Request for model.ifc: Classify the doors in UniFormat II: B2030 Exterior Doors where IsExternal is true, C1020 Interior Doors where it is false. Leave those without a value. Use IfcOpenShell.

First a look at what the model holds.

```python
import ifcopenshell
import ifcopenshell.util.element

model = ifcopenshell.open("model.ifc")
print(model.schema)
print("classifications:", [c.Name for c in model.by_type("IfcClassification")])
values = [ifcopenshell.util.element.get_pset(e, "Pset_DoorCommon", "IsExternal") for e in model.by_type("IfcDoor")]
for value in (True, False, None):
    print("IsExternal", value, values.count(value))
```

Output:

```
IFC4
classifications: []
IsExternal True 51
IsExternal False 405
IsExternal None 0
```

```python
import ifcopenshell
import ifcopenshell.api.classification
import ifcopenshell.util.element

model = ifcopenshell.open("model.ifc")

system = ifcopenshell.api.classification.add_classification(model, classification="UniFormat II")

doors = model.by_type("IfcDoor")
external = {e: ifcopenshell.util.element.get_pset(e, "Pset_DoorCommon", "IsExternal") for e in doors}
for flag, code, name in ((True, "B2030", "Exterior Doors"), (False, "C1020", "Interior Doors")):
    products = [e for e in doors if external[e] is flag]
    ifcopenshell.api.classification.add_reference(
        model, products=products, classification=system, identification=code, name=name
    )
    print(code, len(products))

model.write("model_rev.ifc")
```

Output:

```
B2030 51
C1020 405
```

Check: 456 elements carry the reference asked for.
